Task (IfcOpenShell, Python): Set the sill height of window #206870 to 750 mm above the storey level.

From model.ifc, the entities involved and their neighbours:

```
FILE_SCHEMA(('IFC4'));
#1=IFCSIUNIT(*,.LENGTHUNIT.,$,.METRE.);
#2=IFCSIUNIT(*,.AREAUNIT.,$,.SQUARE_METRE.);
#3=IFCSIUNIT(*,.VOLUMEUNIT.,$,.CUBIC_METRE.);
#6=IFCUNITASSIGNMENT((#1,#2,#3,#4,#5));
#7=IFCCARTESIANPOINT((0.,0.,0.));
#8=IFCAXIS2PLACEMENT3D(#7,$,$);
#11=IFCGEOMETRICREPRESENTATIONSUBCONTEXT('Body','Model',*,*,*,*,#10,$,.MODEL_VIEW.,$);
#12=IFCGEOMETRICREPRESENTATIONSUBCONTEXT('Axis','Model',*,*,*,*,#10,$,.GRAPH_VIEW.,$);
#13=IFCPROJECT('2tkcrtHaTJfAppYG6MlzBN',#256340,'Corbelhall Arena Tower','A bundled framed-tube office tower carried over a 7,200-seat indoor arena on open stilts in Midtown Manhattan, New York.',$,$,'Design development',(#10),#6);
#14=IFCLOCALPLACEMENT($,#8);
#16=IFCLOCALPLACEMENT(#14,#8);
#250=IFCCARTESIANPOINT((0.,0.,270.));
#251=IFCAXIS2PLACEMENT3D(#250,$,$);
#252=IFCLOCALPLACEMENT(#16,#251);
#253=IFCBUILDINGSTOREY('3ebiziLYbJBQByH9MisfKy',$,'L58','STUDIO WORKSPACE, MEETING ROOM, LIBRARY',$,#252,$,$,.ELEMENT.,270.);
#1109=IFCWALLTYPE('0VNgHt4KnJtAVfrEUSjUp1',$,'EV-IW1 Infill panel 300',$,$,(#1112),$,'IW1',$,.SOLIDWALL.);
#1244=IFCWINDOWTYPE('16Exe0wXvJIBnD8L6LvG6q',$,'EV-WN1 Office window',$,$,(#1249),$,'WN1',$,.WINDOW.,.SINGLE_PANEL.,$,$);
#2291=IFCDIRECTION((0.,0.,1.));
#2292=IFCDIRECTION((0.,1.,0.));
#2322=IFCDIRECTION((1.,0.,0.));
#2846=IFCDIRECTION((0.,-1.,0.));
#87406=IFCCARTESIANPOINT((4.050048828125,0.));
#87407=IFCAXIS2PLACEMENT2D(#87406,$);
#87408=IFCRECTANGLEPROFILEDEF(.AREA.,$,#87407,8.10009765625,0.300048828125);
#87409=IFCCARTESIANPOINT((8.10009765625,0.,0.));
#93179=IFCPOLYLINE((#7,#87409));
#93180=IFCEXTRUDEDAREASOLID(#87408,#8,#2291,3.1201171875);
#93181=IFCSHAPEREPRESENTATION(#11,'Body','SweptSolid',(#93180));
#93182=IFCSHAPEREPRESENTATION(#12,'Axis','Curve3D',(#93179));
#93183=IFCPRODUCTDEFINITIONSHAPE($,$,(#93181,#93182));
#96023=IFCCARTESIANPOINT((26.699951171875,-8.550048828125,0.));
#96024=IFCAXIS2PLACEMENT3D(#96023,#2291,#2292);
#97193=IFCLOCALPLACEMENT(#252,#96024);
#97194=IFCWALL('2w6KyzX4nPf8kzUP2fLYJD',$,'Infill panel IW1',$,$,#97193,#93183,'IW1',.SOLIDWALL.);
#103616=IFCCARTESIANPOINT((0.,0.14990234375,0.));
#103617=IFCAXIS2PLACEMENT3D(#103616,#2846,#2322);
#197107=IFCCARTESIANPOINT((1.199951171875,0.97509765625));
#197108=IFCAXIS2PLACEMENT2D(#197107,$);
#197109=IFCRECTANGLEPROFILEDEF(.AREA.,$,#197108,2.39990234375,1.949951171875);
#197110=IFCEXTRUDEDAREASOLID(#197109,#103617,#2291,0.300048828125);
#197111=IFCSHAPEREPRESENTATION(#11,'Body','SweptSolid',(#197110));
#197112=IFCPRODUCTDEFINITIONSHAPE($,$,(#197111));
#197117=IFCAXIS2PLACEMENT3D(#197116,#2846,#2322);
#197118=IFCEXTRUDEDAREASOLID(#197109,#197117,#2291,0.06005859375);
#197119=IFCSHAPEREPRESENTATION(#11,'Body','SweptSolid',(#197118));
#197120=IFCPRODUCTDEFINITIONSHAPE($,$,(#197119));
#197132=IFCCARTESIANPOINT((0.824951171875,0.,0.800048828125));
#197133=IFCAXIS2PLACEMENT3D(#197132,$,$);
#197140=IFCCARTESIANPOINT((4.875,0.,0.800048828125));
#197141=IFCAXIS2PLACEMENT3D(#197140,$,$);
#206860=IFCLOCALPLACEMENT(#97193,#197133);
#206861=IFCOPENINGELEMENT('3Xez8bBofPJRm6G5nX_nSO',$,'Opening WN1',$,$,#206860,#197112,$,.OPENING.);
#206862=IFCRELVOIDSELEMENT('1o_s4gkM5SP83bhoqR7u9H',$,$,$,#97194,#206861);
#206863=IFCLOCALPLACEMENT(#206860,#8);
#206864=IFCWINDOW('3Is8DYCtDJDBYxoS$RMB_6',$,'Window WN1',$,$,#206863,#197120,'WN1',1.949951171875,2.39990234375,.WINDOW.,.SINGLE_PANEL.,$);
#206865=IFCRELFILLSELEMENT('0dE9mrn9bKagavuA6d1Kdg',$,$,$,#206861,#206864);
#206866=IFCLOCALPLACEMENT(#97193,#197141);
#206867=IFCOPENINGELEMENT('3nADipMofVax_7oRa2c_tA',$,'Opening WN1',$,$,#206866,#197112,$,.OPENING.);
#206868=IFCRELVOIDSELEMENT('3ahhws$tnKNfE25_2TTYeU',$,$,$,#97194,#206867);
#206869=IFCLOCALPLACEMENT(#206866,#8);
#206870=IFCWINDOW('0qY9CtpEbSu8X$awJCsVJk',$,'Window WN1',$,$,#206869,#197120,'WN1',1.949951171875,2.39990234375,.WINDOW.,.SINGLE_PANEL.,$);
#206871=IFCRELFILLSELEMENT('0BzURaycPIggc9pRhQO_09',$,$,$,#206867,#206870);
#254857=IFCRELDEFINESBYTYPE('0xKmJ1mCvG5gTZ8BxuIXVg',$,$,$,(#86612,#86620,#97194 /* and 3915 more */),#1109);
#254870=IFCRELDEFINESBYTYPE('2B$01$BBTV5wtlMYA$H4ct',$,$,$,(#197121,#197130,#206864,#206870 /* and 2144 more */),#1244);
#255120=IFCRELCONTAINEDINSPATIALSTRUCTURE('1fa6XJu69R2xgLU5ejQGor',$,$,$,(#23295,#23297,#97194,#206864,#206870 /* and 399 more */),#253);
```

```python
import numpy as np
import ifcopenshell
import ifcopenshell.api.geometry
import ifcopenshell.geom
import ifcopenshell.util.element
import ifcopenshell.util.placement
import ifcopenshell.util.shape
import ifcopenshell.util.unit

model = ifcopenshell.open("model.ifc")
unit_scale = ifcopenshell.util.unit.calculate_unit_scale(model)

window = model.by_id(206870)
opening = window.FillsVoids[0].RelatingOpeningElement
storey = ifcopenshell.util.element.get_container(window, ifc_class="IfcBuildingStorey")
level = ifcopenshell.util.placement.get_local_placement(storey.ObjectPlacement)[2, 3]

# The opening's origin need not be at the sill, so measure its lowest point.
shape = ifcopenshell.geom.create_shape(ifcopenshell.geom.settings(), opening)
bottom = ifcopenshell.util.shape.get_shape_bottom_elevation(shape, shape.geometry) / unit_scale
dz = level + 0.75 - bottom

shift = np.array([0.0, 0.0, dz])
# The window is placed relative to its opening, so it follows when the opening moves.
matrix = ifcopenshell.util.placement.get_local_placement(opening.ObjectPlacement)
matrix[:3, 3] += shift
ifcopenshell.api.geometry.edit_object_placement(
    model, product=opening, matrix=matrix, is_si=False, should_transform_children=True
)

print(f"moved by {dz * unit_scale:+.3f} m")

model.write("model_rev.ifc")
```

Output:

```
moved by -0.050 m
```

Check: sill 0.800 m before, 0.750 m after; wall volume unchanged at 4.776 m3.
